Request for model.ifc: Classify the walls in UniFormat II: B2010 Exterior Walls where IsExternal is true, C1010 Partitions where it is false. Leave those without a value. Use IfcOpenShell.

First a look at what the model holds.

```python
import ifcopenshell
import ifcopenshell.util.element

model = ifcopenshell.open("model.ifc")
print(model.schema)
print("classifications:", [c.Name for c in model.by_type("IfcClassification")])
values = [ifcopenshell.util.element.get_pset(e, "Pset_WallCommon", "IsExternal") for e in model.by_type("IfcWall")]
for value in (True, False, None):
    print("IsExternal", value, values.count(value))
```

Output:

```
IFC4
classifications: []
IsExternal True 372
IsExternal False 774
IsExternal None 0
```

```python
import ifcopenshell
import ifcopenshell.api.classification
import ifcopenshell.util.element

model = ifcopenshell.open("model.ifc")

system = ifcopenshell.api.classification.add_classification(model, classification="UniFormat II")

walls = model.by_type("IfcWall")
external = {e: ifcopenshell.util.element.get_pset(e, "Pset_WallCommon", "IsExternal") for e in walls}
for flag, code, name in ((True, "B2010", "Exterior Walls"), (False, "C1010", "Partitions")):
    products = [e for e in walls if external[e] is flag]
    ifcopenshell.api.classification.add_reference(
        model, products=products, classification=system, identification=code, name=name
    )
    print(code, len(products))

model.write("model_rev.ifc")
```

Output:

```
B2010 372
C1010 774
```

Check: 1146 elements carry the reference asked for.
